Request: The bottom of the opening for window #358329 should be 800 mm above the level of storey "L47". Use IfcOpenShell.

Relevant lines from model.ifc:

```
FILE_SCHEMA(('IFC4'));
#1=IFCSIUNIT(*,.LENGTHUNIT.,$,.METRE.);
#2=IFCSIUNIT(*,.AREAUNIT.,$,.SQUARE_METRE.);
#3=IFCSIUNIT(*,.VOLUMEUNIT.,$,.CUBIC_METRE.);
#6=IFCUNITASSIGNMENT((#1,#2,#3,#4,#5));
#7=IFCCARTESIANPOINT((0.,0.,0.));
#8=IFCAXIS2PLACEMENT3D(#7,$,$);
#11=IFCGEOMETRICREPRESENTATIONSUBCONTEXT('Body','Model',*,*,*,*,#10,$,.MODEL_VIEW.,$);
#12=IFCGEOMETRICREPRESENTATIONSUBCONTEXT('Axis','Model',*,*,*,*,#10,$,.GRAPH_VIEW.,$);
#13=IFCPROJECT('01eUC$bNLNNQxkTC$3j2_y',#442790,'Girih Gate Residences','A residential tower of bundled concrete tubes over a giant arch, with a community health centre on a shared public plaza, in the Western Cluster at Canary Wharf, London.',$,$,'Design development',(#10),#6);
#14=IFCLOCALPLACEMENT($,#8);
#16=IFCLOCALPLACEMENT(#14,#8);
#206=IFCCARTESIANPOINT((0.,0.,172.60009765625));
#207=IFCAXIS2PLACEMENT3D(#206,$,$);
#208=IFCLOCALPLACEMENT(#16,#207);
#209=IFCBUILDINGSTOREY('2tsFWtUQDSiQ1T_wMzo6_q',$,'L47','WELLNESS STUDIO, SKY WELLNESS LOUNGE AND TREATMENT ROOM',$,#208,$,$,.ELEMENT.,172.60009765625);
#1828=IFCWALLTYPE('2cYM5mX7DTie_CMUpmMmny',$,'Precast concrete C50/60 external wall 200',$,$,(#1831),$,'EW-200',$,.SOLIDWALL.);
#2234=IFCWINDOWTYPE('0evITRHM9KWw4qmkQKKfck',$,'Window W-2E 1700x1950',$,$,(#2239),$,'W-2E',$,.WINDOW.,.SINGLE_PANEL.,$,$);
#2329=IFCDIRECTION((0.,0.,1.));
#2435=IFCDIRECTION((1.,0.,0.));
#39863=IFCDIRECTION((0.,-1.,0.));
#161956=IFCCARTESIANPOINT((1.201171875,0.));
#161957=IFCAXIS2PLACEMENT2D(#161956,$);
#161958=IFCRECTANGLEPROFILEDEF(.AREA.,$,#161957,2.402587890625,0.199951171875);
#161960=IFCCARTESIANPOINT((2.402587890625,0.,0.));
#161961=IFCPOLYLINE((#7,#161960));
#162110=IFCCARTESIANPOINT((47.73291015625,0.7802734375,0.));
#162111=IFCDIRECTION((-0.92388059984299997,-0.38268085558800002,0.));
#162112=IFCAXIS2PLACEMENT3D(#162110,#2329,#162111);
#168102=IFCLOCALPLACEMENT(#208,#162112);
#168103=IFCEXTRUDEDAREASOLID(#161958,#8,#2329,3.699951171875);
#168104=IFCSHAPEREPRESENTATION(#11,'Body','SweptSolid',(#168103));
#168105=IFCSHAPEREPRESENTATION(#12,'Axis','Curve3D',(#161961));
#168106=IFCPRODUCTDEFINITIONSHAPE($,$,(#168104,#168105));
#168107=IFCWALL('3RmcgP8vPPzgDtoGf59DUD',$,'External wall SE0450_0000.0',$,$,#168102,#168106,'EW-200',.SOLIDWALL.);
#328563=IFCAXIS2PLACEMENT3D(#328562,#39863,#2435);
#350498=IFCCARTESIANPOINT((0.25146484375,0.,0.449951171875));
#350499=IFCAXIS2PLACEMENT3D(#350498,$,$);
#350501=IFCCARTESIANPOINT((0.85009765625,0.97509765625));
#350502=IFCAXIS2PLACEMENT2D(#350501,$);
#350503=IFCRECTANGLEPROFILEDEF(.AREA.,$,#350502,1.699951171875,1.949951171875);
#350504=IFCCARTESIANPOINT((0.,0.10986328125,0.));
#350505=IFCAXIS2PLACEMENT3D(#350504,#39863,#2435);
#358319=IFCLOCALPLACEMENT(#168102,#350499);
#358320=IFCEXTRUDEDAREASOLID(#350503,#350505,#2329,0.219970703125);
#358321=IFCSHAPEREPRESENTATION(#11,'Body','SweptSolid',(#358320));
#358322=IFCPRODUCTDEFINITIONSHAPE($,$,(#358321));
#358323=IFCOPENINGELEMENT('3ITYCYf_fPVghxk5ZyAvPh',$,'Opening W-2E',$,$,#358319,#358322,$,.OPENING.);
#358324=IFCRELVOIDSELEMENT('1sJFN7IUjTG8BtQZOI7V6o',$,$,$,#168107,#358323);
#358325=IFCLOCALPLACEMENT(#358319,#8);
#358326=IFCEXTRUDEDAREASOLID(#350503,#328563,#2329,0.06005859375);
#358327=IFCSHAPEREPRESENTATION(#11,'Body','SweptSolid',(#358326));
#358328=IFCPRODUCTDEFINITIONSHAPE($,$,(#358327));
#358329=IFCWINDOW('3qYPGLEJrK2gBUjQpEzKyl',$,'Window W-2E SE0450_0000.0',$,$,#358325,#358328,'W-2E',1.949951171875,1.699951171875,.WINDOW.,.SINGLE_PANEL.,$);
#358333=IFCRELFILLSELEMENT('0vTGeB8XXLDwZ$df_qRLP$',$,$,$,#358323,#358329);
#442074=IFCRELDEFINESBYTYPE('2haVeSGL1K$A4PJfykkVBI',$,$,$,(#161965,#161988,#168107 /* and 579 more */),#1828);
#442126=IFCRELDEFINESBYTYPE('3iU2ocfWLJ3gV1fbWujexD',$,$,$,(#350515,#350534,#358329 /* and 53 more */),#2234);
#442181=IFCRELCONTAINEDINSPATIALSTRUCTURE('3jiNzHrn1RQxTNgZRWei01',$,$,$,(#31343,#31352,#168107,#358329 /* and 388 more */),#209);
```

```python
import numpy as np
import ifcopenshell
import ifcopenshell.api.geometry
import ifcopenshell.geom
import ifcopenshell.util.element
import ifcopenshell.util.placement
import ifcopenshell.util.shape
import ifcopenshell.util.unit

model = ifcopenshell.open("model.ifc")
unit_scale = ifcopenshell.util.unit.calculate_unit_scale(model)

window = model.by_id(358329)
opening = window.FillsVoids[0].RelatingOpeningElement
storey = ifcopenshell.util.element.get_container(window, ifc_class="IfcBuildingStorey")
level = ifcopenshell.util.placement.get_local_placement(storey.ObjectPlacement)[2, 3]

# The opening's origin need not be at the sill, so measure its lowest point.
shape = ifcopenshell.geom.create_shape(ifcopenshell.geom.settings(), opening)
bottom = ifcopenshell.util.shape.get_shape_bottom_elevation(shape, shape.geometry) / unit_scale
dz = level + 0.8 / unit_scale - bottom

shift = np.array([0.0, 0.0, dz])
# The window is placed relative to its opening, so it follows when the opening moves.
matrix = ifcopenshell.util.placement.get_local_placement(opening.ObjectPlacement)
matrix[:3, 3] += shift
ifcopenshell.api.geometry.edit_object_placement(
    model, product=opening, matrix=matrix, is_si=False, should_transform_children=True
)

print(f"moved by {dz * unit_scale:+.3f} m")

model.write("model_updated.ifc")
```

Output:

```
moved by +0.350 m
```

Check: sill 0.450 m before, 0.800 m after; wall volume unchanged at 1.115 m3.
